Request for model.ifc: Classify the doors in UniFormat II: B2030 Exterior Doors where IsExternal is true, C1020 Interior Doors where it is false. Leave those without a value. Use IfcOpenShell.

First a look at what the model holds.

```python
import ifcopenshell
import ifcopenshell.util.element

model = ifcopenshell.open("model.ifc")
print(model.schema)
print("classifications:", [c.Name for c in model.by_type("IfcClassification")])
values = [ifcopenshell.util.element.get_pset(e, "Pset_DoorCommon", "IsExternal") for e in model.by_type("IfcDoor")]
for value in (True, False, None):
    print("IsExternal", value, values.count(value))
```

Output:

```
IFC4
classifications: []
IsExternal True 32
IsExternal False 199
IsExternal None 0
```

```python
import ifcopenshell
import ifcopenshell.api.classification
import ifcopenshell.util.element

model = ifcopenshell.open("model.ifc")

system = ifcopenshell.api.classification.add_classification(model, classification="UniFormat II")

doors = model.by_type("IfcDoor")
external = {e: ifcopenshell.util.element.get_pset(e, "Pset_DoorCommon", "IsExternal") for e in doors}
for flag, code, name in ((True, "B2030", "Exterior Doors"), (False, "C1020", "Interior Doors")):
    products = [e for e in doors if external[e] is flag]
    ifcopenshell.api.classification.add_reference(
        model, products=products, classification=system, identification=code, name=name
    )
    print(code, len(products))

model.write("model-out.ifc")
```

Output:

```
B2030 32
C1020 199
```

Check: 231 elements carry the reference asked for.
